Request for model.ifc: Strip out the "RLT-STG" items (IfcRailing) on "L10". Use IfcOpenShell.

First a look at what the model holds.

```python
import ifcopenshell
import ifcopenshell.util.element

model = ifcopenshell.open("model.ifc")
print(model.schema)
storey = next(s for s in model.by_type("IfcBuildingStorey") if s.Name == "L10")
railings = [e for e in ifcopenshell.util.element.get_decomposition(storey) if e.is_a("IfcRailing")]
seen = {}
for e in railings:
    element_type = ifcopenshell.util.element.get_type(e)
    name = element_type.Name if element_type not in (None, e) else None
    seen[name] = seen.get(name, 0) + 1
for name, count in sorted(seen.items(), key=str):
    print(count, "x", name)
```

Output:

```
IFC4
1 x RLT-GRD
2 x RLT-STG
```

```python
import ifcopenshell
import ifcopenshell.api.root
import ifcopenshell.util.element

model = ifcopenshell.open("model.ifc")

storey = next(s for s in model.by_type("IfcBuildingStorey") if s.Name == "L10")
railings = [e for e in ifcopenshell.util.element.get_decomposition(storey) if e.is_a("IfcRailing")]
targets = [e for e in railings if (t := ifcopenshell.util.element.get_type(e)) not in (None, e) and t.Name == "RLT-STG"]

for e in targets:
    ifcopenshell.api.root.remove_product(model, product=e)
print(len(targets), "removed")

model.write("model_rev.ifc")
```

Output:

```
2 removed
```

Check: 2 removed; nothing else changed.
